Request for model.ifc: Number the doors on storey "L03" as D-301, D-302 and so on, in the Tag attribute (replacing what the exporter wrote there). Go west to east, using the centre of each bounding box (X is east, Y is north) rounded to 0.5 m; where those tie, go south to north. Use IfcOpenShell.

First a look at what the model holds.

```python
import ifcopenshell
import ifcopenshell.util.element
import ifcopenshell.util.placement

model = ifcopenshell.open("model.ifc")
print(model.schema)
storey = next(s for s in model.by_type("IfcBuildingStorey") if s.Name == "L03")
doors = [e for e in ifcopenshell.util.element.get_decomposition(storey) if e.is_a("IfcDoor")]
for e in sorted(doors, key=lambda e: e.id()):
    origin = ifcopenshell.util.placement.get_local_placement(e.ObjectPlacement)[:3, 3]
    print(e.id(), e.Tag, e.Name, origin.round(2) + 0.0, sep=" | ")
```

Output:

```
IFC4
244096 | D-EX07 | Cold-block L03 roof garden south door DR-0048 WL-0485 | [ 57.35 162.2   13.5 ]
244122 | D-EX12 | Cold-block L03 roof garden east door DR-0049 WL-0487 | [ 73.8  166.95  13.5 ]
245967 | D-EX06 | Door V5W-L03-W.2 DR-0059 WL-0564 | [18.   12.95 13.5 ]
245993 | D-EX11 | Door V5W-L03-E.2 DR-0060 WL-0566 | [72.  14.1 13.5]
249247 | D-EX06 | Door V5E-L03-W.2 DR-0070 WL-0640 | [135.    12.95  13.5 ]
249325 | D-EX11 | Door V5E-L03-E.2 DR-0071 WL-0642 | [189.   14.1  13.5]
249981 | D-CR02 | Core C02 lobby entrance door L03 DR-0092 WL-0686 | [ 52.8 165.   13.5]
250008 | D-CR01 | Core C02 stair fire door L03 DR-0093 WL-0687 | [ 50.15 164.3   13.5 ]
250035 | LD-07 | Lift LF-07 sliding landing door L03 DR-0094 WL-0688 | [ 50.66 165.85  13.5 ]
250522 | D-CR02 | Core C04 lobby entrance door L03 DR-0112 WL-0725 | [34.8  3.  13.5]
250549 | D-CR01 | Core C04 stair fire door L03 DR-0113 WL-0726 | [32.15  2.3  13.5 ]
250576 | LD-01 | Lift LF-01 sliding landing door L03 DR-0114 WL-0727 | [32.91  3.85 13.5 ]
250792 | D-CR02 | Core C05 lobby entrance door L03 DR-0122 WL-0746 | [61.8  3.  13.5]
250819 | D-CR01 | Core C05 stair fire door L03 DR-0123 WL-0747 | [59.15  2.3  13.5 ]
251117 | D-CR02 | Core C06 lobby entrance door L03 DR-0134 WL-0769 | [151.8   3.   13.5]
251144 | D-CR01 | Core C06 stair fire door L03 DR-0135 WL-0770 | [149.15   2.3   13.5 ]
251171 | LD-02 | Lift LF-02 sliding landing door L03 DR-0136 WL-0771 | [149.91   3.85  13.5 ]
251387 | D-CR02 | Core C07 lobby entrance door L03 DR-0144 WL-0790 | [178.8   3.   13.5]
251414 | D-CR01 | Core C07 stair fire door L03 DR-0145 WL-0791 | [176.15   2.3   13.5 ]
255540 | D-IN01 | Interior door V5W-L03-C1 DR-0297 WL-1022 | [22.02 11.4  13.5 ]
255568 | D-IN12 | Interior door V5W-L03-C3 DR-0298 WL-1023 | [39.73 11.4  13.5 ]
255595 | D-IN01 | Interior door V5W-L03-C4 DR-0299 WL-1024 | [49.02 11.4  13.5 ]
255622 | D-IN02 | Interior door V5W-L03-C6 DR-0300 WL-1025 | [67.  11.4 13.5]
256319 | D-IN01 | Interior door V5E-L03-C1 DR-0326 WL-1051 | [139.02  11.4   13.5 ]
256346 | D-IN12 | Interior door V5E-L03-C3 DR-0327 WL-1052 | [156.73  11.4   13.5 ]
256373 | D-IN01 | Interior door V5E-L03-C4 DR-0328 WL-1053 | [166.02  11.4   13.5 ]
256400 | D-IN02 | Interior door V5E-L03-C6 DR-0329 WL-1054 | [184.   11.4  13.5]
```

```python
import ifcopenshell
import ifcopenshell.geom
import ifcopenshell.util.element
import ifcopenshell.util.shape

model = ifcopenshell.open("model.ifc")
settings = ifcopenshell.geom.settings()
settings.set("use-world-coords", True)


def centre(element):
    shape = ifcopenshell.geom.create_shape(settings, element)
    return ifcopenshell.util.shape.get_bbox_centroid(shape.geometry)


storey = next(s for s in model.by_type("IfcBuildingStorey") if s.Name == "L03")
doors = [e for e in ifcopenshell.util.element.get_decomposition(storey) if e.is_a("IfcDoor")]

# Insertion points can sit at a corner or the storey origin, so sort by the geometry (in metres).
centres = {e: centre(e) for e in doors}
doors.sort(key=lambda e: (round(centres[e][0] / 0.5), centres[e][1]))

for i, e in enumerate(doors, start=1):
    number = f"D-3{i:02d}"
    e.Tag = number
    print(e.id(), number)

model.write("model_rev.ifc")
```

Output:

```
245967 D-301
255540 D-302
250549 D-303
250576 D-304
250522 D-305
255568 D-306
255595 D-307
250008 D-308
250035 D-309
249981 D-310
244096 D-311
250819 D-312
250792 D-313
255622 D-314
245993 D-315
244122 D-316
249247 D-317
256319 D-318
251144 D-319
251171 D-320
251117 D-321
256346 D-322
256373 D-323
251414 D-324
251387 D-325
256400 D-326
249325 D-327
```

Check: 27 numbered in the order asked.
